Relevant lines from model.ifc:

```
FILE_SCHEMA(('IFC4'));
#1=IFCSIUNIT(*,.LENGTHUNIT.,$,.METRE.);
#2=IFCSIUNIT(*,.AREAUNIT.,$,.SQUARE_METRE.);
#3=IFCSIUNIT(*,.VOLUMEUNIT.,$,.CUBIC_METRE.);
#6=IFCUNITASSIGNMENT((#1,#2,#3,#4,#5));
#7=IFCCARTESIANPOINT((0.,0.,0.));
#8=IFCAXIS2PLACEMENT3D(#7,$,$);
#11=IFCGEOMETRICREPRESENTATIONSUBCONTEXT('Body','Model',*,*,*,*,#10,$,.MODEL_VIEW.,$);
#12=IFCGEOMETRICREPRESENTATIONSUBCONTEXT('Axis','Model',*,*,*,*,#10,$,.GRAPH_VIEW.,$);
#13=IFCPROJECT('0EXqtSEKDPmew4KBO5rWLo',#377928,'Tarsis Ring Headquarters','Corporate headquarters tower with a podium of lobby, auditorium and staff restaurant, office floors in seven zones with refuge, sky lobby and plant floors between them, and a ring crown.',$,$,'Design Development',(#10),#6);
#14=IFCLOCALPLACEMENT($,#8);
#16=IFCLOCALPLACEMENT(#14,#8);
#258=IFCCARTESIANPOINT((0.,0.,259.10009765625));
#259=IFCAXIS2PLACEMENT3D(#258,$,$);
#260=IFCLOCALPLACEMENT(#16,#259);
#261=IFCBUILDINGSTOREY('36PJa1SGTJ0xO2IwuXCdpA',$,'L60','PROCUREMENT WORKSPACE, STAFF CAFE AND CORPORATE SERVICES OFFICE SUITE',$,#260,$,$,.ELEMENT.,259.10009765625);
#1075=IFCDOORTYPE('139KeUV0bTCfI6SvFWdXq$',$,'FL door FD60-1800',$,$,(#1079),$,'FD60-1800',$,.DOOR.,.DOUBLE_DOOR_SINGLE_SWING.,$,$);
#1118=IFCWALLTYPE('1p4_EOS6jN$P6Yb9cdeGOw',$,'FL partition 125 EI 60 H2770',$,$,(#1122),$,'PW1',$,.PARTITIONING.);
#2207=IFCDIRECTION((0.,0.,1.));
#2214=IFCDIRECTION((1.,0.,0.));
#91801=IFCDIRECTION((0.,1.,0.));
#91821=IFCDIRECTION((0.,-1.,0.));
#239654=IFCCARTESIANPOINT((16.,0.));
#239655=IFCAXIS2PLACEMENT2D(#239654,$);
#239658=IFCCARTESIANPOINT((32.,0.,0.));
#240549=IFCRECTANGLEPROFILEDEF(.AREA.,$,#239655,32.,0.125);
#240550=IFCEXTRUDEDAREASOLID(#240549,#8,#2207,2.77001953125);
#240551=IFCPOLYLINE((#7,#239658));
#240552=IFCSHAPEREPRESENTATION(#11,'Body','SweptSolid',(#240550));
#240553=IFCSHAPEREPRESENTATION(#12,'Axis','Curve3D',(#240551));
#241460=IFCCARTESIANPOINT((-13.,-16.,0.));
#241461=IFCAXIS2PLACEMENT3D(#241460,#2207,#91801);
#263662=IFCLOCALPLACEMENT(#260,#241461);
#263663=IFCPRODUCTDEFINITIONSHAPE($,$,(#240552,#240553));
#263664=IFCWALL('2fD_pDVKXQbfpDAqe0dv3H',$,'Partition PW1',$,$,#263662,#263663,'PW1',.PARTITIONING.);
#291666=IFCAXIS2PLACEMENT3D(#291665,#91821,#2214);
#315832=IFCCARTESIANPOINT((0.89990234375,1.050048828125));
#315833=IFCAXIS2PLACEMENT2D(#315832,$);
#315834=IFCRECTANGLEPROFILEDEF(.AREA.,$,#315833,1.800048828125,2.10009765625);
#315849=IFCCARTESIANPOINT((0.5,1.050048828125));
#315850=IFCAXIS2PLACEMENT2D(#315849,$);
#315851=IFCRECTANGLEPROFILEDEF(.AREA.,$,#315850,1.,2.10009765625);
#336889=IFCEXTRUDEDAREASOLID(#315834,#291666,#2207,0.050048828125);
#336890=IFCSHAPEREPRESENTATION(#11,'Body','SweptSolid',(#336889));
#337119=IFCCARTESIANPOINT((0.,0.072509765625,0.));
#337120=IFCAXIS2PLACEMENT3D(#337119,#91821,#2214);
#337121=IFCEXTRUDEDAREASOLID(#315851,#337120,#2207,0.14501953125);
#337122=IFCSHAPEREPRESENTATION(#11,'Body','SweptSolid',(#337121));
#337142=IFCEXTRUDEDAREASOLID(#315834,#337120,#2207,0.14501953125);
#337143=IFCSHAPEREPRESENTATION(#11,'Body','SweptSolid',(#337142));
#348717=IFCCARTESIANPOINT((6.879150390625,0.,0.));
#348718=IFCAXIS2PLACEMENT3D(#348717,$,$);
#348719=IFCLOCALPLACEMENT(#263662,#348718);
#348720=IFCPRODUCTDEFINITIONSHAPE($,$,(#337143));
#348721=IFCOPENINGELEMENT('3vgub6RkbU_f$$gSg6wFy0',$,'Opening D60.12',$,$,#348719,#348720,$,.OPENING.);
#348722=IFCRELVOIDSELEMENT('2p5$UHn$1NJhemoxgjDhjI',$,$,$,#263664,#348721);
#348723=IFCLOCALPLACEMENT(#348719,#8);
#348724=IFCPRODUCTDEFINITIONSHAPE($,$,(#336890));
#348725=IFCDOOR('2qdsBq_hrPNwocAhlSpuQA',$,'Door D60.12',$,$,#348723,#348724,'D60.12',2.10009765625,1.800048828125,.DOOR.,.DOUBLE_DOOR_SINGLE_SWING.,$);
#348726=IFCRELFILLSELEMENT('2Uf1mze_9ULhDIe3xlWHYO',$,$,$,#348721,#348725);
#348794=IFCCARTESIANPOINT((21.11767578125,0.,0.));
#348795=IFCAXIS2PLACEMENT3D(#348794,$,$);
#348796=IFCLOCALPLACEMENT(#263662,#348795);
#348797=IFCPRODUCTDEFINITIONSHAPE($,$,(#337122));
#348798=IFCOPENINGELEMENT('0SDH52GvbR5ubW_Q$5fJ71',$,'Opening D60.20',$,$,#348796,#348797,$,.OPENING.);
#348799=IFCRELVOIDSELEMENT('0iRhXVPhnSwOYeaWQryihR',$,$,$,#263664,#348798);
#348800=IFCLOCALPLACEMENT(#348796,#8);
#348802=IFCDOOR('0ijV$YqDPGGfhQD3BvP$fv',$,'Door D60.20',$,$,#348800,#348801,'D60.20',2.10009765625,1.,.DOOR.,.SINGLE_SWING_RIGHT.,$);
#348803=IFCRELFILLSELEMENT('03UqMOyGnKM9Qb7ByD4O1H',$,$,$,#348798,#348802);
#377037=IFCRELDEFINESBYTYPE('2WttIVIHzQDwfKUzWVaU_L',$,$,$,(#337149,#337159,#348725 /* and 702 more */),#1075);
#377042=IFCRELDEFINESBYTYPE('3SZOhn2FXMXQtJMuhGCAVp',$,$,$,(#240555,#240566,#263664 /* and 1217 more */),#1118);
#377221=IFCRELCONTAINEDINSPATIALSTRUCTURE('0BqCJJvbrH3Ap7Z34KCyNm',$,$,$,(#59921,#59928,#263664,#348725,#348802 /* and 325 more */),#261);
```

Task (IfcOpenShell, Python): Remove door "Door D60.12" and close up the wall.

```python
import ifcopenshell
import ifcopenshell.api.feature
import ifcopenshell.api.root
import ifcopenshell.geom
import ifcopenshell.util.shape

model = ifcopenshell.open("model.ifc")
settings = ifcopenshell.geom.settings()


def volume(element):
    """Net volume in cubic metres, openings subtracted."""
    shape = ifcopenshell.geom.create_shape(settings, element)
    return ifcopenshell.util.shape.get_volume(shape.geometry)


door = model.by_guid("2qdsBq_hrPNwocAhlSpuQA")
opening = door.FillsVoids[0].RelatingOpeningElement
wall = opening.VoidsElements[0].RelatingBuildingElement
before = volume(wall)

ifcopenshell.api.root.remove_product(model, product=door)
ifcopenshell.api.feature.remove_feature(model, feature=opening)

after = volume(wall)

print(f"wall volume {before:.3f} -> {after:.3f} m3")

model.write("model_updated.ifc")
```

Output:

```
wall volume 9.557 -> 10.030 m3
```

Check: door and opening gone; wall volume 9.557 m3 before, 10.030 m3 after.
